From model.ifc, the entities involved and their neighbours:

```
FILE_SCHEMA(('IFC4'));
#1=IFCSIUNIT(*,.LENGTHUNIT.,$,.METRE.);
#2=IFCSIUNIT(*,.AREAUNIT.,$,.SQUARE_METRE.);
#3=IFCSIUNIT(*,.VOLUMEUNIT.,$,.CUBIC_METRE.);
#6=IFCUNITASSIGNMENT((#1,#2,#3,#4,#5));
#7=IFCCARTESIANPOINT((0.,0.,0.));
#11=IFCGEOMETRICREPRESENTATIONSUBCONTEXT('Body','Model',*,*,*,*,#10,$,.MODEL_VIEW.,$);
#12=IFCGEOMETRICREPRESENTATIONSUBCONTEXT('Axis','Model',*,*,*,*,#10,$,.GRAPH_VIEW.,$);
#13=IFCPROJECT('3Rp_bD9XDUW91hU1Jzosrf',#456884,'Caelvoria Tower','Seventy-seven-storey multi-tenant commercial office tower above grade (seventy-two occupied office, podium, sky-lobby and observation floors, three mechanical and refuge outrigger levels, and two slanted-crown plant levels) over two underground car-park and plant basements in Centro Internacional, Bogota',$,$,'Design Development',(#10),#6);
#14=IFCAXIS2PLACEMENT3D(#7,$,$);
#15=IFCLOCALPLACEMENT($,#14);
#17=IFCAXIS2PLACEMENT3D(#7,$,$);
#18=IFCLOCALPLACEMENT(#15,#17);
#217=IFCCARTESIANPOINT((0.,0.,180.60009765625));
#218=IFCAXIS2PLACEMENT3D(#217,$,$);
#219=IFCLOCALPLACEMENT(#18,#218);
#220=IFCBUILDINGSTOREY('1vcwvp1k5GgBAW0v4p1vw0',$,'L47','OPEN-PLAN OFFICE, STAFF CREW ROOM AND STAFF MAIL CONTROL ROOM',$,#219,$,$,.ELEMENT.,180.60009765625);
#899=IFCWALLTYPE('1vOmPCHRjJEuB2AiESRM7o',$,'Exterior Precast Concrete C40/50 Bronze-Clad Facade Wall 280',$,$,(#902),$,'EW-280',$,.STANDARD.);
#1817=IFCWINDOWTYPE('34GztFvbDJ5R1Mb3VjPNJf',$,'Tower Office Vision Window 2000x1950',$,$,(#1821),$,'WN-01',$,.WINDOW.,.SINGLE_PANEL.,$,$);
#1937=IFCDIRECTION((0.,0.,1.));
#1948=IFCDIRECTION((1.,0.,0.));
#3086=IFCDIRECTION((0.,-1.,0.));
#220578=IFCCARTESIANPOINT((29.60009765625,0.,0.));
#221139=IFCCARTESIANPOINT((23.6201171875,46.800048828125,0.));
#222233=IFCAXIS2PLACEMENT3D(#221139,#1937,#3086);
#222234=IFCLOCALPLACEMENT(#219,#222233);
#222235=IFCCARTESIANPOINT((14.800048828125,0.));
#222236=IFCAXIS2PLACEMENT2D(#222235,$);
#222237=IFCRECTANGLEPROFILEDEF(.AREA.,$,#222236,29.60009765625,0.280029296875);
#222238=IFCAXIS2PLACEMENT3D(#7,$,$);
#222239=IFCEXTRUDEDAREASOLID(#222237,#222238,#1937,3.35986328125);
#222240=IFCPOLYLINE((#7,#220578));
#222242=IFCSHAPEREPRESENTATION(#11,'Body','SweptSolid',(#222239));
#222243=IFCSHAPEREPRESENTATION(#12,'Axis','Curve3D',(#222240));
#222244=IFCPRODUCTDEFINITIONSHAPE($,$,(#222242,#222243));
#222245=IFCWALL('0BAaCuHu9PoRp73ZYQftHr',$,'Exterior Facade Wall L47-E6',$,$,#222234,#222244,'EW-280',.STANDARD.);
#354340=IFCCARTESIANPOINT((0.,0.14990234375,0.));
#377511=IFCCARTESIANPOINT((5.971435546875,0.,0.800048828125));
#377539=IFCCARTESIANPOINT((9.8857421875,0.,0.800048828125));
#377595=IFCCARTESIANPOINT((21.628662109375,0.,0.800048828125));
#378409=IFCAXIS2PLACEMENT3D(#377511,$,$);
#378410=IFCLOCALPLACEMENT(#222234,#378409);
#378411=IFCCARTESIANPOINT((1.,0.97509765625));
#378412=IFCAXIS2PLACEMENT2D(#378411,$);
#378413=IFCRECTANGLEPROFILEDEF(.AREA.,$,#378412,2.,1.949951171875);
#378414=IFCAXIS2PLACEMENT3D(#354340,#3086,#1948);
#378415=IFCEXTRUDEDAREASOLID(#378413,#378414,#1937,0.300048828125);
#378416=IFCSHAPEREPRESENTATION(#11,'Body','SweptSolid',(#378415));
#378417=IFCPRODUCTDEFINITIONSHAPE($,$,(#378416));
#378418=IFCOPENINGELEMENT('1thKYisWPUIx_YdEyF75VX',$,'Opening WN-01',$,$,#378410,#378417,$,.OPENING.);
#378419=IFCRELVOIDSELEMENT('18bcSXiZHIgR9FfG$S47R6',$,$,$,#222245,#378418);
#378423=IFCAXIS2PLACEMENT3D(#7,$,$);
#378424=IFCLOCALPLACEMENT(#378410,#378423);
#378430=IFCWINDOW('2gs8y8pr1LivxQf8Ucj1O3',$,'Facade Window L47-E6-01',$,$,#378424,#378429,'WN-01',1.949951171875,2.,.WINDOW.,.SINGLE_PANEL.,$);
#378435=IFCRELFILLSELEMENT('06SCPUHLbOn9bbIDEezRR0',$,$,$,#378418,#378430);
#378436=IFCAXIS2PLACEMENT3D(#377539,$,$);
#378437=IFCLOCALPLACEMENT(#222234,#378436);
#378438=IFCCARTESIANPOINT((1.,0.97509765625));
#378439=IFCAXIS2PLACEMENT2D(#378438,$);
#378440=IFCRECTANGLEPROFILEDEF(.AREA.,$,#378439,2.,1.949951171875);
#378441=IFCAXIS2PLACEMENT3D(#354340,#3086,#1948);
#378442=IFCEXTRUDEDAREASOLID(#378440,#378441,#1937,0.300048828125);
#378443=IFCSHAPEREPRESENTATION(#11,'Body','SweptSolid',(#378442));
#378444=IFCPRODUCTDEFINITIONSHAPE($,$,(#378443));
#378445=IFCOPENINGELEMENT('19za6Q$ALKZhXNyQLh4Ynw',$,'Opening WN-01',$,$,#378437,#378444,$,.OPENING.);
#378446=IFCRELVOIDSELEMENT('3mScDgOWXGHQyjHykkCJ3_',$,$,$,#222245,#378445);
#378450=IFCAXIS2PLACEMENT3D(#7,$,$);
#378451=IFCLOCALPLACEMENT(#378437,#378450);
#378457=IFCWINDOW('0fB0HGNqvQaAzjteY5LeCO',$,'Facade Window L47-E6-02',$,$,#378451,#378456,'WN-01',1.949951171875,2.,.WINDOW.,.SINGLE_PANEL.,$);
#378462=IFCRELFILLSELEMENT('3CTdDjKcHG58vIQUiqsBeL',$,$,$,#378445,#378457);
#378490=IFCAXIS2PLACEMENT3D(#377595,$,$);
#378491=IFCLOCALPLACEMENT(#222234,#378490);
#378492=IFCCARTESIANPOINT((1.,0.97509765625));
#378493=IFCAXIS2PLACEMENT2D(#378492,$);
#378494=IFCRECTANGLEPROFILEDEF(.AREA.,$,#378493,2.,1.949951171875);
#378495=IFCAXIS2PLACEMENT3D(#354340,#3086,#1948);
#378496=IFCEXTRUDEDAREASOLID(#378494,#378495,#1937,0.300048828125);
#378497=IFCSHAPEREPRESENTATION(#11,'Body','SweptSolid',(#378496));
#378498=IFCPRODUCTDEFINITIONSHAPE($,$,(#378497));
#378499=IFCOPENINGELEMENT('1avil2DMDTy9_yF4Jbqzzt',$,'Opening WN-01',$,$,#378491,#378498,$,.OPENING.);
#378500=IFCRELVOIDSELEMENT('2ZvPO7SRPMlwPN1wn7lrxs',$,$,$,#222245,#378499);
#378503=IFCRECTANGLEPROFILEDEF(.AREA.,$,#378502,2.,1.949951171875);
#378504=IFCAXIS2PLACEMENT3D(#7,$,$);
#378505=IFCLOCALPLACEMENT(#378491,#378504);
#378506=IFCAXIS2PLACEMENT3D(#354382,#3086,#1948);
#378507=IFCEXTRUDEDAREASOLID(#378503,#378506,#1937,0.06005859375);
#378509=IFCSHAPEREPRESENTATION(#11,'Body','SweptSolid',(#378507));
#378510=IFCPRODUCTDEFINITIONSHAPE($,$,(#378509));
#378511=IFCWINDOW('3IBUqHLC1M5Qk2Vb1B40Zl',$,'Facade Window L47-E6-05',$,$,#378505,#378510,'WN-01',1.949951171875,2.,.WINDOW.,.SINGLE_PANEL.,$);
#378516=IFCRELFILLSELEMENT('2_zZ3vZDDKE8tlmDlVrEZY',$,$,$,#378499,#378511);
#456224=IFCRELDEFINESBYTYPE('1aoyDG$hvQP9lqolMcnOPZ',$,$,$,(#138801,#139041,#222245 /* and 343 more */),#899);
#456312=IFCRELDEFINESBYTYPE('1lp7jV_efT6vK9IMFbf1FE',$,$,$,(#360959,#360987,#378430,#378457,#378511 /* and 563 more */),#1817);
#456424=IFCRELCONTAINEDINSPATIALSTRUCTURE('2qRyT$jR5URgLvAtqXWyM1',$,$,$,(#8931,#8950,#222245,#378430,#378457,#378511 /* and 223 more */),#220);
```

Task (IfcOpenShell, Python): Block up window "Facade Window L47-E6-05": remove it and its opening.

```python
import ifcopenshell
import ifcopenshell.api.feature
import ifcopenshell.api.root
import ifcopenshell.geom
import ifcopenshell.util.shape

model = ifcopenshell.open("model.ifc")
settings = ifcopenshell.geom.settings()


def volume(element):
    """Net volume in cubic metres, openings subtracted."""
    shape = ifcopenshell.geom.create_shape(settings, element)
    return ifcopenshell.util.shape.get_volume(shape.geometry)


window = model.by_guid("3IBUqHLC1M5Qk2Vb1B40Zl")
opening = window.FillsVoids[0].RelatingOpeningElement
wall = opening.VoidsElements[0].RelatingBuildingElement
before = volume(wall)

ifcopenshell.api.root.remove_product(model, product=window)
ifcopenshell.api.feature.remove_feature(model, feature=opening)

after = volume(wall)

print(f"wall volume {before:.3f} -> {after:.3f} m3")

model.write("model_updated.ifc")
```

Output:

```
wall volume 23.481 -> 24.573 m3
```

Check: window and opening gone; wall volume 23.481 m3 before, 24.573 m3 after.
